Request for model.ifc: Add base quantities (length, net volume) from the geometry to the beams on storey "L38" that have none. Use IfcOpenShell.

First a look at what the model holds.

```python
import ifcopenshell
import ifcopenshell.util.element
import ifcopenshell.util.unit

model = ifcopenshell.open("model.ifc")
print(model.schema)
for unit_type in ("LENGTHUNIT", "AREAUNIT", "VOLUMEUNIT"):
    print(unit_type, ifcopenshell.util.unit.calculate_unit_scale(model, unit_type))
storey = next(s for s in model.by_type("IfcBuildingStorey") if s.Name == "L38")
beams = [e for e in ifcopenshell.util.element.get_decomposition(storey) if e.is_a("IfcBeam")]
for e in sorted(beams, key=lambda e: e.id()):
    print(e.id(), e.is_a(), e.Name, list(ifcopenshell.util.element.get_psets(e, qtos_only=True)), sep=" | ")
```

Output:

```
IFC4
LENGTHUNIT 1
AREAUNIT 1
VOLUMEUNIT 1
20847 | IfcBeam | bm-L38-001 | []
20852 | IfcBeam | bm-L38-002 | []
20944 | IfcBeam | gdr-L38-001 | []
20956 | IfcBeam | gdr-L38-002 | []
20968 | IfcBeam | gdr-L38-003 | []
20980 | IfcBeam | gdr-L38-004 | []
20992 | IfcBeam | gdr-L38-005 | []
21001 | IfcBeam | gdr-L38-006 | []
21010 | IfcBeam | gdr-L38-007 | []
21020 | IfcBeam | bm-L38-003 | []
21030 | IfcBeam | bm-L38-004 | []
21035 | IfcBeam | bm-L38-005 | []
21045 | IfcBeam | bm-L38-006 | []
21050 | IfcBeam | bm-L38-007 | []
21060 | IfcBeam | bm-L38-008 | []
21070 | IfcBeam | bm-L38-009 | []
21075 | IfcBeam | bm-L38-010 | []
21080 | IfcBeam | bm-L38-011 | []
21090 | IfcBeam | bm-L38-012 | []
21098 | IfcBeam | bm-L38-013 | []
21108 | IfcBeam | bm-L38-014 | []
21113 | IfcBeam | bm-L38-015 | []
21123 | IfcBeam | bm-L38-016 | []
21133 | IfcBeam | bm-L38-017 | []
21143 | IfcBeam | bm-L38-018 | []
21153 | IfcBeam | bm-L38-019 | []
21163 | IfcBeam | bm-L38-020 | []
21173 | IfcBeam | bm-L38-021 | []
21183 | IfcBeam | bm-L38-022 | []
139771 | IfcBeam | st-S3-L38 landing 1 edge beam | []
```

```python
import ifcopenshell
import ifcopenshell.api.pset
import ifcopenshell.geom
import ifcopenshell.util.element
import ifcopenshell.util.shape
import ifcopenshell.util.unit

model = ifcopenshell.open("model.ifc")
unit_scale = ifcopenshell.util.unit.calculate_unit_scale(model)
volume_scale = ifcopenshell.util.unit.calculate_unit_scale(model, "VOLUMEUNIT")
settings = ifcopenshell.geom.settings()

storey = next(s for s in model.by_type("IfcBuildingStorey") if s.Name == "L38")
beams = [e for e in ifcopenshell.util.element.get_decomposition(storey) if e.is_a("IfcBeam")]

for e in sorted(beams, key=lambda e: e.id()):
    if ifcopenshell.util.element.get_psets(e, qtos_only=True, should_inherit=False):
        continue
    # Geometry comes back in metres, in the element's own axes.
    shape = ifcopenshell.geom.create_shape(settings, e)
    values = {
        "Length": ifcopenshell.util.shape.get_max_xyz(shape.geometry) / unit_scale,
        "NetVolume": ifcopenshell.util.shape.get_volume(shape.geometry) / volume_scale,
    }
    qto = ifcopenshell.api.pset.add_qto(model, product=e, name="Qto_BeamBaseQuantities")
    ifcopenshell.api.pset.edit_qto(model, qto=qto, properties=values)
    print(e.id(), {k: round(v, 3) for k, v in values.items()})

model.write("model_edited.ifc")
```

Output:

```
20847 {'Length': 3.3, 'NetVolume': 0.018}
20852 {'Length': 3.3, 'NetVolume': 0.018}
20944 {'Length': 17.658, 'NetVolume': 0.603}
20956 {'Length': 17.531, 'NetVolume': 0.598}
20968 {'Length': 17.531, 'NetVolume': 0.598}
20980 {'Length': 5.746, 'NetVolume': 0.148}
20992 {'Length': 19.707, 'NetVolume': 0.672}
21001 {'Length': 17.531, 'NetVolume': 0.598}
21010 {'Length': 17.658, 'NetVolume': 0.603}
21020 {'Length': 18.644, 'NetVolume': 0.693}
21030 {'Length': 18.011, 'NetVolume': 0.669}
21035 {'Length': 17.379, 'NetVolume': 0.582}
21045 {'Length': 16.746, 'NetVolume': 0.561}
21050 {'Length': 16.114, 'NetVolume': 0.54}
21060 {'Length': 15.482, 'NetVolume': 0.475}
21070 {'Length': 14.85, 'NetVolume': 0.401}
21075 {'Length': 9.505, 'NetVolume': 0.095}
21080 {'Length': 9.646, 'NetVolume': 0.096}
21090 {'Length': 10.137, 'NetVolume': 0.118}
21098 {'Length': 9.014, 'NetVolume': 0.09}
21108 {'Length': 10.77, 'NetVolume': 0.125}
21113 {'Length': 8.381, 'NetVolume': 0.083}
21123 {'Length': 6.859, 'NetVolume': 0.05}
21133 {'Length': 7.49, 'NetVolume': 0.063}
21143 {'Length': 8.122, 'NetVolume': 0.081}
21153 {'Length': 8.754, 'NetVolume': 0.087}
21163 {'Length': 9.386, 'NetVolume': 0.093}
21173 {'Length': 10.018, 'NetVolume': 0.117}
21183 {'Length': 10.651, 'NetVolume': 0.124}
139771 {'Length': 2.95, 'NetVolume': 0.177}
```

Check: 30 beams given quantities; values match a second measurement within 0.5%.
